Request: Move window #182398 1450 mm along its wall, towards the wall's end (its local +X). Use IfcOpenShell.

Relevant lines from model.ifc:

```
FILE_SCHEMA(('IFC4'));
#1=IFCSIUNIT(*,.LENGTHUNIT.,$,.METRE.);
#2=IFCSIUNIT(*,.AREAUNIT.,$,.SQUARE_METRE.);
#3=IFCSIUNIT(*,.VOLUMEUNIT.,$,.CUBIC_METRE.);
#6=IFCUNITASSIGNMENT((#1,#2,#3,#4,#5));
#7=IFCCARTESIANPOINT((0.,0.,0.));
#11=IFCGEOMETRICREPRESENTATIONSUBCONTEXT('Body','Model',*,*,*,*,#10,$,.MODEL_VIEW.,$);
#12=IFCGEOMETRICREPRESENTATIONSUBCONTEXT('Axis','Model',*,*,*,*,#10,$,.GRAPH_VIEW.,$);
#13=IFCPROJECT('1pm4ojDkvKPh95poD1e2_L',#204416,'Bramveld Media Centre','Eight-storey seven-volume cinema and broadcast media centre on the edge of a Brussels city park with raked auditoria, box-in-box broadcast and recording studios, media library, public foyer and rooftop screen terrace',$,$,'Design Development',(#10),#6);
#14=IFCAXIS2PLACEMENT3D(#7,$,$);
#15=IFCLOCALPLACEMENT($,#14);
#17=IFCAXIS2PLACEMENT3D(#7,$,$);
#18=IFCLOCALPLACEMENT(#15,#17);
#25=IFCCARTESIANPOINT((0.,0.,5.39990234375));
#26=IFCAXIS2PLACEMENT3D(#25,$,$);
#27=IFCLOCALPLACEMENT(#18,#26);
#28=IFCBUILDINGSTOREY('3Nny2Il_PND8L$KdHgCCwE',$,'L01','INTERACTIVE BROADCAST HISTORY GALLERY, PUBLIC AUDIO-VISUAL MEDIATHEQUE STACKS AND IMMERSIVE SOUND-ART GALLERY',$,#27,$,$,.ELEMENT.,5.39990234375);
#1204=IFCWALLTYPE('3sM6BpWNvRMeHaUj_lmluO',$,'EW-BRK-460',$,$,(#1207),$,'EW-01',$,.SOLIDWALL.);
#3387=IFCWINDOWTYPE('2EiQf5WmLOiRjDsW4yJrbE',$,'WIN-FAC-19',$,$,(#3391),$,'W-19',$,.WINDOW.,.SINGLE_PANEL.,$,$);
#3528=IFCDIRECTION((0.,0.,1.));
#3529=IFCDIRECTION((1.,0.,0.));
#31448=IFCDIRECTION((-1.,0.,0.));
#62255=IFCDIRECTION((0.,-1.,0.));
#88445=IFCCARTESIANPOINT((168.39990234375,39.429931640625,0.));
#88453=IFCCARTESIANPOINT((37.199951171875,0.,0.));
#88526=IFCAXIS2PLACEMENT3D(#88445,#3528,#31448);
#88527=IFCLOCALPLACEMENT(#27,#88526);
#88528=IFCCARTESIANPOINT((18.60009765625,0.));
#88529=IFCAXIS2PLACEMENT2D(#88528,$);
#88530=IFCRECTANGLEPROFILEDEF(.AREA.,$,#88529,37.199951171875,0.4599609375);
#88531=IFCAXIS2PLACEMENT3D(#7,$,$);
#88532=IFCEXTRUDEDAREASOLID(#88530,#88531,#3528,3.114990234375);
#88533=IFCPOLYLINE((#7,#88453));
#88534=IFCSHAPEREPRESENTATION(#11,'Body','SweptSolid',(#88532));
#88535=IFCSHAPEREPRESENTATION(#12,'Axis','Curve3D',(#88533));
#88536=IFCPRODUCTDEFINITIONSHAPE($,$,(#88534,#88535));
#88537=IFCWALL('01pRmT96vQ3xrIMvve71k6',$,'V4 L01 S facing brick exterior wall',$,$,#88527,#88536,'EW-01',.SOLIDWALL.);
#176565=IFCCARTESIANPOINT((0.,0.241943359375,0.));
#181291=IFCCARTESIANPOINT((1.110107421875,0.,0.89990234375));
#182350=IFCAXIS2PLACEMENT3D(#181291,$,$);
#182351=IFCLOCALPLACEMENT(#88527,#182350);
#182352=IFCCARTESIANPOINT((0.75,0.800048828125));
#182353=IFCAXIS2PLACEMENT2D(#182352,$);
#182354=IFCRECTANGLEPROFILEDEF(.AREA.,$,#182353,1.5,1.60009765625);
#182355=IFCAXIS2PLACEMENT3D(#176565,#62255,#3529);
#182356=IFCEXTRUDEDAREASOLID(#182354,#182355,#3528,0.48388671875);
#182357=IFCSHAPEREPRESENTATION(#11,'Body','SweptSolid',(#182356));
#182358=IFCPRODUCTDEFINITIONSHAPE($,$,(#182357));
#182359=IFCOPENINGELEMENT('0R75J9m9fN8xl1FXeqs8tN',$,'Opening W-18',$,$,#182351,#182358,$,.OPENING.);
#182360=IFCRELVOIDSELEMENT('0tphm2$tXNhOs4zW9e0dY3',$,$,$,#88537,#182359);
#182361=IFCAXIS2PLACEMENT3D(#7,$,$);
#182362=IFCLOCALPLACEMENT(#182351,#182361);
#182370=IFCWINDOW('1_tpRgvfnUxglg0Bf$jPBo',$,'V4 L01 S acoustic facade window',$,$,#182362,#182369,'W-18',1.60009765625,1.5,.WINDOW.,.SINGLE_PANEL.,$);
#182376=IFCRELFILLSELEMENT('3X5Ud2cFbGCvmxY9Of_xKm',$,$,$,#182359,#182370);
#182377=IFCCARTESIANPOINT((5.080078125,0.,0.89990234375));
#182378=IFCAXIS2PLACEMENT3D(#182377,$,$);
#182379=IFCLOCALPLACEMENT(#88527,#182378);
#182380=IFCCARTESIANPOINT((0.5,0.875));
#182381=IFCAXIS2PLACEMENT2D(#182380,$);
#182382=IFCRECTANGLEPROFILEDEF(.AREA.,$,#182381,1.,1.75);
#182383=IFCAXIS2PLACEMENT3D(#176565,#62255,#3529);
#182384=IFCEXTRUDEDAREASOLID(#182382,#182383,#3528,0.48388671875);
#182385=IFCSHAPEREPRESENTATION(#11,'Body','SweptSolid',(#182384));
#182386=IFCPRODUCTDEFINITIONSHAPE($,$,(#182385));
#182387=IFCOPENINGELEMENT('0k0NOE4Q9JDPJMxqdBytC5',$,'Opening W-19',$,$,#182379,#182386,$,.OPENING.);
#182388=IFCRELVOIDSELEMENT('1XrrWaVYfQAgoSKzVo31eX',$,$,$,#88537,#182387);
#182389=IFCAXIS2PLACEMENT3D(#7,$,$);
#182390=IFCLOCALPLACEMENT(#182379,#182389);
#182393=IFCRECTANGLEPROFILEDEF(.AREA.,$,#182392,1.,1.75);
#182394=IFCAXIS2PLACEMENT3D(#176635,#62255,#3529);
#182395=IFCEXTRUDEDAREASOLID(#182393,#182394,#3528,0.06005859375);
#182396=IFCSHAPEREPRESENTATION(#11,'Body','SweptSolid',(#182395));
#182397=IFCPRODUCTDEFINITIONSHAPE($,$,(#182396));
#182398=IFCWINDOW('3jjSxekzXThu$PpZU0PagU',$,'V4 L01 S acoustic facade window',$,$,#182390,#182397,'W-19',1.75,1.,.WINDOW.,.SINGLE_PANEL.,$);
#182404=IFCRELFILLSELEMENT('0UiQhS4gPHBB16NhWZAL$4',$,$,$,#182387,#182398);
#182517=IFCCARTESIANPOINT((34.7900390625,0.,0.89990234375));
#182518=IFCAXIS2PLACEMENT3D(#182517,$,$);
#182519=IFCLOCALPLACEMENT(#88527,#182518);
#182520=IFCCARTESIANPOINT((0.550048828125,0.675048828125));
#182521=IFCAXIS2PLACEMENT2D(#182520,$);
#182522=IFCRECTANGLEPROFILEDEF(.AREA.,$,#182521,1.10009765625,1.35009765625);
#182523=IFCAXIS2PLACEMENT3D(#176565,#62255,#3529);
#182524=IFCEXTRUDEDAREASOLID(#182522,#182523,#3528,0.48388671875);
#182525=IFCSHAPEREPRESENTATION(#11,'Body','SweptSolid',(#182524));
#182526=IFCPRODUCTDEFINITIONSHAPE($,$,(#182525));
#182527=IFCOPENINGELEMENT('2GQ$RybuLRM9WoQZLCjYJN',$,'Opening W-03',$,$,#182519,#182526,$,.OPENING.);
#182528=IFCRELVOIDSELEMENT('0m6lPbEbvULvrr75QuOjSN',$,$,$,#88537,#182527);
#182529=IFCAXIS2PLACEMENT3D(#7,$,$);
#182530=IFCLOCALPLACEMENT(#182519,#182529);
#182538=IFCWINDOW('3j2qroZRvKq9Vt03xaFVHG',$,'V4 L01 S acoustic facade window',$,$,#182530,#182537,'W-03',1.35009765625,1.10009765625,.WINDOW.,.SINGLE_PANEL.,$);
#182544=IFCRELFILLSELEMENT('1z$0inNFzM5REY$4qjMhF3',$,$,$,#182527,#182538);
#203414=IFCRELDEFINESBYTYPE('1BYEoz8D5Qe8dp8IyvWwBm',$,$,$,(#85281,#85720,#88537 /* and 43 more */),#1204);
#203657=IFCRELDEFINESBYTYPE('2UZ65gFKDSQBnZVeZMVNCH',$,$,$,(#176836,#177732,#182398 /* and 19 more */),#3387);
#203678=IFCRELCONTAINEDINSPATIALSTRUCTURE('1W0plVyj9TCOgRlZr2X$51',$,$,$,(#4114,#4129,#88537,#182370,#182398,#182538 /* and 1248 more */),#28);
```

```python
import ifcopenshell
import ifcopenshell.api.geometry
import ifcopenshell.util.placement

model = ifcopenshell.open("model.ifc")

window = model.by_guid("3jjSxekzXThu$PpZU0PagU")
opening = window.FillsVoids[0].RelatingOpeningElement
wall = opening.VoidsElements[0].RelatingBuildingElement

wall_matrix = ifcopenshell.util.placement.get_local_placement(wall.ObjectPlacement)
shift = wall_matrix[:3, 0] * 1.45
before = ifcopenshell.util.placement.get_local_placement(window.ObjectPlacement)[:3, 3].copy()

# The window is placed relative to its opening, so it follows when the opening moves.
matrix = ifcopenshell.util.placement.get_local_placement(opening.ObjectPlacement)
matrix[:3, 3] += shift
ifcopenshell.api.geometry.edit_object_placement(
    model, product=opening, matrix=matrix, is_si=False, should_transform_children=True
)

after = ifcopenshell.util.placement.get_local_placement(window.ObjectPlacement)[:3, 3]
print("window moved by", (after - before).round(3) + 0.0)

model.write("model_rev.ifc")
```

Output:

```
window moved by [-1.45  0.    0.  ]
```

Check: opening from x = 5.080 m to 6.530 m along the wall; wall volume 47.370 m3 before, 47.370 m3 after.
